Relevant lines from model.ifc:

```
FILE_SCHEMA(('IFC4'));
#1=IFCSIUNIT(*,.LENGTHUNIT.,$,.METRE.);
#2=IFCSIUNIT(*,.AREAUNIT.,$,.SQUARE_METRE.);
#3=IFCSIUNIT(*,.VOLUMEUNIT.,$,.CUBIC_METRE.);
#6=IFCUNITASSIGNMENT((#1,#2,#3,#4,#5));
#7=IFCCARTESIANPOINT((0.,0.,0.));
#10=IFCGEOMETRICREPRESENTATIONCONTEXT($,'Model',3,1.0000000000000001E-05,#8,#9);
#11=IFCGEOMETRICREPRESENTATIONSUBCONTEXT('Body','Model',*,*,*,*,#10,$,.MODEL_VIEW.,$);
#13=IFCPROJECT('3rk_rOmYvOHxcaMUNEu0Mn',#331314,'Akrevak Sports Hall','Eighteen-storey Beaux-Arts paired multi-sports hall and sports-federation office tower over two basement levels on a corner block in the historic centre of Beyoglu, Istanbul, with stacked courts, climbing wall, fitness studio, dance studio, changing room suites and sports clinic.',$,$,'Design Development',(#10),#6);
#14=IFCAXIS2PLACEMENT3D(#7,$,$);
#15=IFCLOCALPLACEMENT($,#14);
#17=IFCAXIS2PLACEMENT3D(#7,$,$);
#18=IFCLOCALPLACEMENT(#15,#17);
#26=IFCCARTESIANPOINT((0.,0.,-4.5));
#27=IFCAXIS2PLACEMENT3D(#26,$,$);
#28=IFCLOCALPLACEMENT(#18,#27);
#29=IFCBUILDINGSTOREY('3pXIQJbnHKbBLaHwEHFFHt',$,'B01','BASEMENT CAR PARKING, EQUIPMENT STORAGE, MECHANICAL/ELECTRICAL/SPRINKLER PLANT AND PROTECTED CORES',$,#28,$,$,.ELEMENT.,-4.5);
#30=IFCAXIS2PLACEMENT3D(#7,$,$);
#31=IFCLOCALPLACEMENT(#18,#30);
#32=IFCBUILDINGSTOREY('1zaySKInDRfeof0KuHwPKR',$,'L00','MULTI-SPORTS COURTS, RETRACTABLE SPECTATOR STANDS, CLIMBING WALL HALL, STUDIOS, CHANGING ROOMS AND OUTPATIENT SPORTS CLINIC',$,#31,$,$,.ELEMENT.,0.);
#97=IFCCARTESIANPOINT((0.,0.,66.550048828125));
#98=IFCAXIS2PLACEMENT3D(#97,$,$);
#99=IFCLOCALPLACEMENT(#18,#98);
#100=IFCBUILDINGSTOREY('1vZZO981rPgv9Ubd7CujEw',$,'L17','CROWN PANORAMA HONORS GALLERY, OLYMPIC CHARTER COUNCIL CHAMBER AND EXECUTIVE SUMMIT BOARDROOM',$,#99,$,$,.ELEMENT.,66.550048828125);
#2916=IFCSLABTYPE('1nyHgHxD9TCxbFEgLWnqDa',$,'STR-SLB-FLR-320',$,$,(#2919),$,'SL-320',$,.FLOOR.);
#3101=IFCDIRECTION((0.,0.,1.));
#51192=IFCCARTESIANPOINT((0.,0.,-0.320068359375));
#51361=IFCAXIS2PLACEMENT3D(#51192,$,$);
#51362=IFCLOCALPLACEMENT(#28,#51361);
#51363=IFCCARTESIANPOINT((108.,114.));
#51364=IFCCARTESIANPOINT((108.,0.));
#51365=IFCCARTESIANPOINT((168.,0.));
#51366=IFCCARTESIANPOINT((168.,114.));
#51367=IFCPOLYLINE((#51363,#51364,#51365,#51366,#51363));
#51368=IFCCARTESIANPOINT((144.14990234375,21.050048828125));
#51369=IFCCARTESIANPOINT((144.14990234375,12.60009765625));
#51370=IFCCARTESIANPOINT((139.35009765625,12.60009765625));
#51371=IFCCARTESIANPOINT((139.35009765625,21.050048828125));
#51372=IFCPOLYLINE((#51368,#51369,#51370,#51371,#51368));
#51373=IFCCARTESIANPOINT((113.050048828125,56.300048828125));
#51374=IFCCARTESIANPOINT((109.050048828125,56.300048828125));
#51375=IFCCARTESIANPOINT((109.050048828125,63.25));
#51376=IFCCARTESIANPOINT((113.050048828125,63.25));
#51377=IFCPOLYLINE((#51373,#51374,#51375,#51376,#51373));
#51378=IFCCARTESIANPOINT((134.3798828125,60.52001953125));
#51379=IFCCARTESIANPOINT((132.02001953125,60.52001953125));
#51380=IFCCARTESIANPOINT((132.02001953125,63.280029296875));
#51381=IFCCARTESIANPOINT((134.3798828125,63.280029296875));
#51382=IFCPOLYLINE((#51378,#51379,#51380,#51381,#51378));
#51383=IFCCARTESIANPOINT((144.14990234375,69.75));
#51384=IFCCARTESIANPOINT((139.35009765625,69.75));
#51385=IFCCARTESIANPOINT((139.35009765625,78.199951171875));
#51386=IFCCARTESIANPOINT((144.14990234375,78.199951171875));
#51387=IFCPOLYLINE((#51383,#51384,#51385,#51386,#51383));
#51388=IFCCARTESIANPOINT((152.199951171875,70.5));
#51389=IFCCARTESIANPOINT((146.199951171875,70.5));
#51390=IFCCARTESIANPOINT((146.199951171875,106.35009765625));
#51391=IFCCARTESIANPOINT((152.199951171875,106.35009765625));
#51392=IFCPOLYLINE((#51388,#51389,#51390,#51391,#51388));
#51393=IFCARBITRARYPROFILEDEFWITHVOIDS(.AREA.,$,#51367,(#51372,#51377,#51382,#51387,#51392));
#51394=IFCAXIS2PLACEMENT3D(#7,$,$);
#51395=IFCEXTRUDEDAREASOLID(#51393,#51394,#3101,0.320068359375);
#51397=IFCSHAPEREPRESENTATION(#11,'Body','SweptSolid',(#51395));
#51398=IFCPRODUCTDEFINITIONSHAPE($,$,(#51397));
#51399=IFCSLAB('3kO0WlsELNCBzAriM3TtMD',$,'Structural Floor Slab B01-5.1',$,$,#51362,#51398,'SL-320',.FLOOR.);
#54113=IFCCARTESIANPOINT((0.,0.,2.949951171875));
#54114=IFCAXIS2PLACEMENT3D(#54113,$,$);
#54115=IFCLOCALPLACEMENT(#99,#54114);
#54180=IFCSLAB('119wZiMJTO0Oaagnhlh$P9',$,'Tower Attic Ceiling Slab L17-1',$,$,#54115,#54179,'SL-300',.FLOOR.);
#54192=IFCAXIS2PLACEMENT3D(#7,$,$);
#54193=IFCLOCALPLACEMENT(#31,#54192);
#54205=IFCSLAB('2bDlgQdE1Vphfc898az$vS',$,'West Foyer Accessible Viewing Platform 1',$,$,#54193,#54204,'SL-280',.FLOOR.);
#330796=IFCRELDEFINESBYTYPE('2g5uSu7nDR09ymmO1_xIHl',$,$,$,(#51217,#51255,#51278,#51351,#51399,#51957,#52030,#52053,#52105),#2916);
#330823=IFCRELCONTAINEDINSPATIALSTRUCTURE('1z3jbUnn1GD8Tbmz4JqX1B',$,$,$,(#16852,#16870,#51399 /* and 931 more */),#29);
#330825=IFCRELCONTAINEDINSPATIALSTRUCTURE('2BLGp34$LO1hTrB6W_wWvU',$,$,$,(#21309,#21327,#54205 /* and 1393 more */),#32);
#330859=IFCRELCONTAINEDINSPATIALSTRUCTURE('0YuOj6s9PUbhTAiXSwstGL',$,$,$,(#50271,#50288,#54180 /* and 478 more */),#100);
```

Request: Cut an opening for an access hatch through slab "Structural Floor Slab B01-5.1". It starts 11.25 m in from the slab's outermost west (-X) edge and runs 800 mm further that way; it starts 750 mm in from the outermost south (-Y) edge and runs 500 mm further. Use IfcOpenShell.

```python
import numpy as np
import ifcopenshell
import ifcopenshell.api.feature
import ifcopenshell.api.geometry
import ifcopenshell.api.root
import ifcopenshell.geom
import ifcopenshell.util.placement
import ifcopenshell.util.representation
import ifcopenshell.util.shape
import ifcopenshell.util.unit

model = ifcopenshell.open("model.ifc")
unit_scale = ifcopenshell.util.unit.calculate_unit_scale(model)
settings = ifcopenshell.geom.settings()


def volume(element):
    """Net volume in cubic metres, openings subtracted."""
    shape = ifcopenshell.geom.create_shape(settings, element)
    return ifcopenshell.util.shape.get_volume(shape.geometry)


slab = model.by_guid("3kO0WlsELNCBzAriM3TtMD")
before = volume(slab)

# Extent in the slab's own axes, in metres. The edges named are its -X and -Y sides.
slab_shape = ifcopenshell.geom.create_shape(settings, slab)
vertices = ifcopenshell.util.shape.get_vertices(slab_shape.geometry)
x_min, y_min, bottom = vertices.min(axis=0)
top = vertices[:, 2].max()

opening = ifcopenshell.api.root.create_entity(model, ifc_class="IfcOpeningElement", name="Access hatch opening", predefined_type="OPENING")
context = ifcopenshell.util.representation.get_context(model, "Model", "Body", "MODEL_VIEW")
width, depth = 0.8, 0.5
outline = [(0.0, 0.0), (width, 0.0), (width, depth), (0.0, depth), (0.0, 0.0)]
# Overshoot both faces by 50 mm so the cut is clean.
shape = ifcopenshell.api.geometry.add_slab_representation(
    model, context=context, depth=top - bottom + 0.1, polyline=outline
)
ifcopenshell.api.geometry.assign_representation(model, product=opening, representation=shape)

matrix = ifcopenshell.util.placement.get_local_placement(slab.ObjectPlacement)
matrix[:, 3] = matrix @ np.append(np.array([x_min + 11.25, y_min + 0.75, bottom - 0.05]) / unit_scale, 1.0)
ifcopenshell.api.geometry.edit_object_placement(model, product=opening, matrix=matrix, is_si=False)
ifcopenshell.api.feature.add_feature(model, feature=opening, element=slab)

after = volume(slab)

print(f"slab volume {before:.3f} -> {after:.3f} m3")

model.write("model_edited.ifc")
```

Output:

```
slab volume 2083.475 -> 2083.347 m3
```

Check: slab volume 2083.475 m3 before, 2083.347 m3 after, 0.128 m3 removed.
